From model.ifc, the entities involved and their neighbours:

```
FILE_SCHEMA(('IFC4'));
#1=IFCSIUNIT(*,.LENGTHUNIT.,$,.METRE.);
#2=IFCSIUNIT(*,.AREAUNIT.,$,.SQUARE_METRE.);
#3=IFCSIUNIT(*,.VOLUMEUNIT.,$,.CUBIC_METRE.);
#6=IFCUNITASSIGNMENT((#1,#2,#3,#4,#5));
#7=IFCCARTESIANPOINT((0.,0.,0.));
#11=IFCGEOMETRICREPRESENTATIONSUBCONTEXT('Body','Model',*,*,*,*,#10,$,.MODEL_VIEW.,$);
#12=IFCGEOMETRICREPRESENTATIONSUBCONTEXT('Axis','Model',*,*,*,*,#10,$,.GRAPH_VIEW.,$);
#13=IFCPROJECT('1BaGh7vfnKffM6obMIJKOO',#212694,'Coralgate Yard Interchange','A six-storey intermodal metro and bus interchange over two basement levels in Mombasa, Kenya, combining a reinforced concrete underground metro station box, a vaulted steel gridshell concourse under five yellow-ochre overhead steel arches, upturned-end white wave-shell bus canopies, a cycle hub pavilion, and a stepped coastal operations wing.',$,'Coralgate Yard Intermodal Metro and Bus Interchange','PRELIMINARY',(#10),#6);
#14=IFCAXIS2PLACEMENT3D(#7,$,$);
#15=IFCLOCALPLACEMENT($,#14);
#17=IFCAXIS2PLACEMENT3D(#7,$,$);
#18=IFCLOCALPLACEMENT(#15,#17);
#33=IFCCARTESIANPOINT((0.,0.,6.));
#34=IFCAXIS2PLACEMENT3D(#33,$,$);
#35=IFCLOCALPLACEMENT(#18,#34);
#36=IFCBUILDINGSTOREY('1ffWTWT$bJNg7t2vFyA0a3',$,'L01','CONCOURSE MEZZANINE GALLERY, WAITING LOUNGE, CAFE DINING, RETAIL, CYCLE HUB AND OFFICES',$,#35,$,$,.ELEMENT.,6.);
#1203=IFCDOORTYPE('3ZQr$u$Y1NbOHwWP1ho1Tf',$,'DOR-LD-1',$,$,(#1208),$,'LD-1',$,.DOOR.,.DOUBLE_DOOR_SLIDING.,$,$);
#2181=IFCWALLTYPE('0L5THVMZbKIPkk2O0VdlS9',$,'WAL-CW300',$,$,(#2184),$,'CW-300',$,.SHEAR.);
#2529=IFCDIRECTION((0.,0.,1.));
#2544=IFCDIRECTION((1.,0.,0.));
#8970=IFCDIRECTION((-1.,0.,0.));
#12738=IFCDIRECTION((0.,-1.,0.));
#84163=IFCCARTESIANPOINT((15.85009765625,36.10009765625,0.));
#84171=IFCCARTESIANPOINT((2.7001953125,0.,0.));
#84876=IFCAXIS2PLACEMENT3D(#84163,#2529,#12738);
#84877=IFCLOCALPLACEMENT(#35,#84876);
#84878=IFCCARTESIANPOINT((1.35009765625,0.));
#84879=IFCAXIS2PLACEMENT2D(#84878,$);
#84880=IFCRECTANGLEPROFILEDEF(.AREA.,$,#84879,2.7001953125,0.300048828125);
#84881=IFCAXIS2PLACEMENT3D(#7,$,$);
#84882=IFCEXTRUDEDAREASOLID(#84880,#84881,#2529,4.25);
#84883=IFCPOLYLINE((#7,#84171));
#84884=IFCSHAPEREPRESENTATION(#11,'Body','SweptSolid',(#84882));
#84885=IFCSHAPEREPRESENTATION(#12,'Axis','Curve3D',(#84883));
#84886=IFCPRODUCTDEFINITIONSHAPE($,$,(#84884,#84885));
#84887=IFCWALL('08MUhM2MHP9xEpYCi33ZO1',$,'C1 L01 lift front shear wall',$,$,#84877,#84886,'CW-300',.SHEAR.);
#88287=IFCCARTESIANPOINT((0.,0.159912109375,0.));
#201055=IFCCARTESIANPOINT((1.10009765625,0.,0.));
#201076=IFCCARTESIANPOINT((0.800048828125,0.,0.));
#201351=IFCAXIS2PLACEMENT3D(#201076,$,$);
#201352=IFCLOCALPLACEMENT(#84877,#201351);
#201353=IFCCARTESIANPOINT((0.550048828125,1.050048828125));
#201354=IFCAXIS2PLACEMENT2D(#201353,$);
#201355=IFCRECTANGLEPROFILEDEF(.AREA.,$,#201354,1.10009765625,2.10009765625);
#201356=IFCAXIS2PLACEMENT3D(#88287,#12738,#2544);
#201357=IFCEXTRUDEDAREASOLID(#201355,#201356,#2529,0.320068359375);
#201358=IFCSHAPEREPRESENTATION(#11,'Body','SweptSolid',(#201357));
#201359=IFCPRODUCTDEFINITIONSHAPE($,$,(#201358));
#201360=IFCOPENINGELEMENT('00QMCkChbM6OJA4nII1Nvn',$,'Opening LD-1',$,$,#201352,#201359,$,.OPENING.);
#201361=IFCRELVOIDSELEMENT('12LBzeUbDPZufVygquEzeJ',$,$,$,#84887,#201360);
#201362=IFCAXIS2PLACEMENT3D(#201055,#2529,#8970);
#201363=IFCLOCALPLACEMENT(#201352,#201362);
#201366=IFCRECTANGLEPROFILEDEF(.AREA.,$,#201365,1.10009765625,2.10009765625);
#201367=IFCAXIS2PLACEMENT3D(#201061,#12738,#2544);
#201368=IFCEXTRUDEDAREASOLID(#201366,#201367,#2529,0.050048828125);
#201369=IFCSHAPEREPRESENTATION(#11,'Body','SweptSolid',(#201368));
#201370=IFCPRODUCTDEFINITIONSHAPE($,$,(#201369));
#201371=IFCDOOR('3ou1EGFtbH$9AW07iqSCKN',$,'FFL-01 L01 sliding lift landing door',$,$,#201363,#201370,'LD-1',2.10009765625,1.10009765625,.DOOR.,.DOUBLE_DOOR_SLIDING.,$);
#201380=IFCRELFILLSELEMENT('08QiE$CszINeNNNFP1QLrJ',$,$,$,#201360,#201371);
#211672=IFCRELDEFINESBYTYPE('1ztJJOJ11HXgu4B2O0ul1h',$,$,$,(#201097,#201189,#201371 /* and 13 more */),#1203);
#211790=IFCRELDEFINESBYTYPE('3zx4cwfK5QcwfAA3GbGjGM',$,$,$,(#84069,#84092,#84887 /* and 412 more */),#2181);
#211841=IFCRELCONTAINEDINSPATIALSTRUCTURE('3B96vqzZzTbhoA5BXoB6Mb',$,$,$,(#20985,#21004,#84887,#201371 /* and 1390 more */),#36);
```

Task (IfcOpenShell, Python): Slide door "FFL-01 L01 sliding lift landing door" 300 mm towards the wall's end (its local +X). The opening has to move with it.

```python
import ifcopenshell
import ifcopenshell.api.geometry
import ifcopenshell.util.placement
import ifcopenshell.util.unit

model = ifcopenshell.open("model.ifc")
unit_scale = ifcopenshell.util.unit.calculate_unit_scale(model)

door = model.by_id(201371)
opening = door.FillsVoids[0].RelatingOpeningElement
wall = opening.VoidsElements[0].RelatingBuildingElement

wall_matrix = ifcopenshell.util.placement.get_local_placement(wall.ObjectPlacement)
shift = wall_matrix[:3, 0] * 0.3 / unit_scale
before = ifcopenshell.util.placement.get_local_placement(door.ObjectPlacement)[:3, 3].copy()

# The door is placed relative to its opening, so it follows when the opening moves.
matrix = ifcopenshell.util.placement.get_local_placement(opening.ObjectPlacement)
matrix[:3, 3] += shift
ifcopenshell.api.geometry.edit_object_placement(
    model, product=opening, matrix=matrix, is_si=False, should_transform_children=True
)

after = ifcopenshell.util.placement.get_local_placement(door.ObjectPlacement)[:3, 3]
print("door moved by", (after - before).round(3) + 0.0)

model.write("model_updated.ifc")
```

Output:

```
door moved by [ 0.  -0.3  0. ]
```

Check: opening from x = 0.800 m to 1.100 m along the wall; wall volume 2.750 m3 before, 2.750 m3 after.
